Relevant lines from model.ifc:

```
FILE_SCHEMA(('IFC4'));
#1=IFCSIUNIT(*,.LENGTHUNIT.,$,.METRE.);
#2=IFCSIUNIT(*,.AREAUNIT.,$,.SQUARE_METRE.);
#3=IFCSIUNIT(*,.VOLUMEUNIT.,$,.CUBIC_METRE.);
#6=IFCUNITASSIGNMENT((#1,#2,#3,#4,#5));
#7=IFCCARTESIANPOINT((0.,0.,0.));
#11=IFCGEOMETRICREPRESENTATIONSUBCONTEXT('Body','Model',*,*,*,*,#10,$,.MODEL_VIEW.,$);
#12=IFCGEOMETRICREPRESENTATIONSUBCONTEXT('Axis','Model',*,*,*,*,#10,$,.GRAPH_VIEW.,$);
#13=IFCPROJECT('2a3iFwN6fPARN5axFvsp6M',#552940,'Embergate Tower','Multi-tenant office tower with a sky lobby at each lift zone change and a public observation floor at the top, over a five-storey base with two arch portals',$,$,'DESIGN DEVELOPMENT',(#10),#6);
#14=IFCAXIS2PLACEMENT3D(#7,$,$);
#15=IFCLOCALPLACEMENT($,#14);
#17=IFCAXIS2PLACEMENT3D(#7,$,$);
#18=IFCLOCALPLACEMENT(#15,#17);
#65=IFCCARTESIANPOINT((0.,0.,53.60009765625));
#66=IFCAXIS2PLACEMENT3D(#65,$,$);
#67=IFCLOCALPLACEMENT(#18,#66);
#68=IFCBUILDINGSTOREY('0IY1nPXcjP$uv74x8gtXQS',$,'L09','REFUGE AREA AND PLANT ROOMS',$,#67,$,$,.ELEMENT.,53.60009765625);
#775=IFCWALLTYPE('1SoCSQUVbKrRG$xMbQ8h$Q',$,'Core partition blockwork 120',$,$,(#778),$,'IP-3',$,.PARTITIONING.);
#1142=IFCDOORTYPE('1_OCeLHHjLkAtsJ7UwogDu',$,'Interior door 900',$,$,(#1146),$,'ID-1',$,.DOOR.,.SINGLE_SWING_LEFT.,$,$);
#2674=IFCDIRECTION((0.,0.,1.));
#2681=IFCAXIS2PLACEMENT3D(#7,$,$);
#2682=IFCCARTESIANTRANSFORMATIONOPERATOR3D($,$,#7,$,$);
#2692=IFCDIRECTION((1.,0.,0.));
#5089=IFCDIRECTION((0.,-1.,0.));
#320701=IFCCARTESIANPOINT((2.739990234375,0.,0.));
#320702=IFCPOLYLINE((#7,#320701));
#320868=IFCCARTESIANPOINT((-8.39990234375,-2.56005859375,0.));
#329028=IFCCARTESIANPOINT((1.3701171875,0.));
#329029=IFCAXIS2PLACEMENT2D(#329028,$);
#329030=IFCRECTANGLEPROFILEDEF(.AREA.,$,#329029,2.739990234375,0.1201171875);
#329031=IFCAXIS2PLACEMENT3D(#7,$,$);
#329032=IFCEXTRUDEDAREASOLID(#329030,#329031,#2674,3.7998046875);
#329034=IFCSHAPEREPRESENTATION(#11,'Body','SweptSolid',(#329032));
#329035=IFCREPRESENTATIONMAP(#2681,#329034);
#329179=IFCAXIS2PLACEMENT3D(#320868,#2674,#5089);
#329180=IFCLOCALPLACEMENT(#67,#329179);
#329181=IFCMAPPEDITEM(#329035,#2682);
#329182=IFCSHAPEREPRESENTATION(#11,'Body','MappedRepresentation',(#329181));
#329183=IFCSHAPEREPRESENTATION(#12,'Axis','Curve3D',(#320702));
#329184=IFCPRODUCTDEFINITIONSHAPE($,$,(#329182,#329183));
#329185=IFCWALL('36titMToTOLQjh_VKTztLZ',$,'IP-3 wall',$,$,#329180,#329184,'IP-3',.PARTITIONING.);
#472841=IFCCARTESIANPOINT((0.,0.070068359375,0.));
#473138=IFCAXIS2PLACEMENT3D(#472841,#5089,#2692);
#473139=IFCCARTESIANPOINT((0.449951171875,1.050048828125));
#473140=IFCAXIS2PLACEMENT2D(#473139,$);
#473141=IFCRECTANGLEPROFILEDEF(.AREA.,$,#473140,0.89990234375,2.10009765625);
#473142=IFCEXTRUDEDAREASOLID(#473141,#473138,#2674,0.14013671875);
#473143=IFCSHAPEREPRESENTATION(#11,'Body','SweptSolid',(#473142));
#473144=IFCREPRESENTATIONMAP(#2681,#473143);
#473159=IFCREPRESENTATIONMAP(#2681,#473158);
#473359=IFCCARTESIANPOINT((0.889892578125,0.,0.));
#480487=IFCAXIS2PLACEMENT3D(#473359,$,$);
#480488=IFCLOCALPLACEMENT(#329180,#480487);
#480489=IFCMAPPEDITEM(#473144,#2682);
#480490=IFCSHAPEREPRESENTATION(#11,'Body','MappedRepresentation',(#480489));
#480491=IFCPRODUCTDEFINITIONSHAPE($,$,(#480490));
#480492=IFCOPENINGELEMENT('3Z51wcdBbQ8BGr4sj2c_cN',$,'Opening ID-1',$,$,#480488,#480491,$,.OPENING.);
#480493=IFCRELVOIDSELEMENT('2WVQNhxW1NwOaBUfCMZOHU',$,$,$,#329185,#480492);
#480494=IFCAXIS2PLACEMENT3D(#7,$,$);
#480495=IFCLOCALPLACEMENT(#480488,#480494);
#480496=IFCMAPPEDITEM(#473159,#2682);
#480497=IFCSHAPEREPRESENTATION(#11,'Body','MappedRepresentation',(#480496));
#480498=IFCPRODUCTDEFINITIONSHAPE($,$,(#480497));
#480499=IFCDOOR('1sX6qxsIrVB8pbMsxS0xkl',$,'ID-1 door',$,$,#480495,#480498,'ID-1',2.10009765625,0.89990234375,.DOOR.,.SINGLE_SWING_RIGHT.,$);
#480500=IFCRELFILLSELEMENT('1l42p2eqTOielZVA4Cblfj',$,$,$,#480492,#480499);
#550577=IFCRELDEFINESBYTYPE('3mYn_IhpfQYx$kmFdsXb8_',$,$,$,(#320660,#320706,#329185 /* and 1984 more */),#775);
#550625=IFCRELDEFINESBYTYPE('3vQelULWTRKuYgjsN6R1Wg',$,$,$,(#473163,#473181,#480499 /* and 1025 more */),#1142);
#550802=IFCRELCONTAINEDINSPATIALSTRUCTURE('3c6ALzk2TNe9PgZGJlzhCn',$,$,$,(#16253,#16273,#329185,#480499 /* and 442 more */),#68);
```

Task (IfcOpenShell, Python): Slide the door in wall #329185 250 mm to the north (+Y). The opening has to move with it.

```python
import ifcopenshell
import ifcopenshell.api.geometry
import ifcopenshell.util.placement
import ifcopenshell.util.unit

model = ifcopenshell.open("model.ifc")
unit_scale = ifcopenshell.util.unit.calculate_unit_scale(model)

door = model.by_id(480499)
opening = door.FillsVoids[0].RelatingOpeningElement
wall = opening.VoidsElements[0].RelatingBuildingElement

wall_matrix = ifcopenshell.util.placement.get_local_placement(wall.ObjectPlacement)
shift = wall_matrix[:3, 0] * -0.25 / unit_scale
before = ifcopenshell.util.placement.get_local_placement(door.ObjectPlacement)[:3, 3].copy()

# The door is placed relative to its opening, so it follows when the opening moves.
matrix = ifcopenshell.util.placement.get_local_placement(opening.ObjectPlacement)
matrix[:3, 3] += shift
ifcopenshell.api.geometry.edit_object_placement(
    model, product=opening, matrix=matrix, is_si=False, should_transform_children=True
)

after = ifcopenshell.util.placement.get_local_placement(door.ObjectPlacement)[:3, 3]
print("door moved by", (after - before).round(3) + 0.0)

model.write("model-out.ifc")
```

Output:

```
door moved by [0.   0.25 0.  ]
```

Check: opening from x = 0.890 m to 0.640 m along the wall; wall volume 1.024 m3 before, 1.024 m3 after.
